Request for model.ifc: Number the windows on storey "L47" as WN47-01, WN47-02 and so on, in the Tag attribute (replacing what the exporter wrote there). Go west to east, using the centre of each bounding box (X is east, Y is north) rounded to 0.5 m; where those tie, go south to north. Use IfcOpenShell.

First a look at what the model holds.

```python
import ifcopenshell
import ifcopenshell.util.element
import ifcopenshell.util.placement

model = ifcopenshell.open("model.ifc")
print(model.schema)
storey = next(s for s in model.by_type("IfcBuildingStorey") if s.Name == "L47")
windows = [e for e in ifcopenshell.util.element.get_decomposition(storey) if e.is_a("IfcWindow")]
for e in sorted(windows, key=lambda e: e.id()):
    origin = ifcopenshell.util.placement.get_local_placement(e.ObjectPlacement)[:3, 3]
    print(e.id(), e.Tag, e.Name, origin.round(2) + 0.0, sep=" | ")
```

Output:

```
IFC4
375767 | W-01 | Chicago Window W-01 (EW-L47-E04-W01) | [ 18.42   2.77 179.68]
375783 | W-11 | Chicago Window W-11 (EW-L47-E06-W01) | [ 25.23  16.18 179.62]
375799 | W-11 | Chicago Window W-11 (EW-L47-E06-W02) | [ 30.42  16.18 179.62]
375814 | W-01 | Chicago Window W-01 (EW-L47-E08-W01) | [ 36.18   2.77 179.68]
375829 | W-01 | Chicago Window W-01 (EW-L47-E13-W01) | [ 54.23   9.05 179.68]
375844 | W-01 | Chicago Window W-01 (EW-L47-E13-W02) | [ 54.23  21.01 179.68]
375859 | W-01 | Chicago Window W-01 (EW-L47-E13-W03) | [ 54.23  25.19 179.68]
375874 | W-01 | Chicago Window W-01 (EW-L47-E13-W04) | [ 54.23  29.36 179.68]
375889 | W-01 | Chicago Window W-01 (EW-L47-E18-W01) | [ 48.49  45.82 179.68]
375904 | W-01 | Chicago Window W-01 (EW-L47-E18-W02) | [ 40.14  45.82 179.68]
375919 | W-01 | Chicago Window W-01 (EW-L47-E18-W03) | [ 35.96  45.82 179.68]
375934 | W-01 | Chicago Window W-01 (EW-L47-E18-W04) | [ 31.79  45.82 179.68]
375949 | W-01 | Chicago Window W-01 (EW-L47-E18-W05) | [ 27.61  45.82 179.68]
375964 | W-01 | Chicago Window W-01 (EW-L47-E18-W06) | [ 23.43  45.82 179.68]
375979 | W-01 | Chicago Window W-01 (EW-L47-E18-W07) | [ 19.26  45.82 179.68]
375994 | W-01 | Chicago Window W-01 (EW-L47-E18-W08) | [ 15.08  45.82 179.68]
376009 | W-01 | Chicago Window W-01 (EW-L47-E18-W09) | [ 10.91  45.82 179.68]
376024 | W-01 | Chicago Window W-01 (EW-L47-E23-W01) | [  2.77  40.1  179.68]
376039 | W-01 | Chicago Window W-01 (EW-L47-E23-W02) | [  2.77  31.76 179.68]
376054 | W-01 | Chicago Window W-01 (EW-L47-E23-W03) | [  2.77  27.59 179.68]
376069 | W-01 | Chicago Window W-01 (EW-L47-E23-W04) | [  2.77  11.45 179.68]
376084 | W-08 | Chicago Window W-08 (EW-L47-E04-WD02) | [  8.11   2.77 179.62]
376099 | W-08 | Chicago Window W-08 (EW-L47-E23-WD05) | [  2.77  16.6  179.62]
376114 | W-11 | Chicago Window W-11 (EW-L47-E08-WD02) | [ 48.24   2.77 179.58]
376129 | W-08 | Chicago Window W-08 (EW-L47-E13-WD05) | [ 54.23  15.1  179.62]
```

```python
import ifcopenshell
import ifcopenshell.geom
import ifcopenshell.util.element
import ifcopenshell.util.shape

model = ifcopenshell.open("model.ifc")
settings = ifcopenshell.geom.settings()
settings.set("use-world-coords", True)


def centre(element):
    shape = ifcopenshell.geom.create_shape(settings, element)
    return ifcopenshell.util.shape.get_bbox_centroid(shape.geometry)


storey = next(s for s in model.by_type("IfcBuildingStorey") if s.Name == "L47")
windows = [e for e in ifcopenshell.util.element.get_decomposition(storey) if e.is_a("IfcWindow")]

# Insertion points can sit at a corner or the storey origin, so sort by the geometry (in metres).
centres = {e: centre(e) for e in windows}
windows.sort(key=lambda e: (round(centres[e][0] / 0.5), centres[e][1]))

for i, e in enumerate(windows, start=1):
    number = f"WN47-{i:02d}"
    e.Tag = number
    print(e.id(), number)

model.write("model-out.ifc")
```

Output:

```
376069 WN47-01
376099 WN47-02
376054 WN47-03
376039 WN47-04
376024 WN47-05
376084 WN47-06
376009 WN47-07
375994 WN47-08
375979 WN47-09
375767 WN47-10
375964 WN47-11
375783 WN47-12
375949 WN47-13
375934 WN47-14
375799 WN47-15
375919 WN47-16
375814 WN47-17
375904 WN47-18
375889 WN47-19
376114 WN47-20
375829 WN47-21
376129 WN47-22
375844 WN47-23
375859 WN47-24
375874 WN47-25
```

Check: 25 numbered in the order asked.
